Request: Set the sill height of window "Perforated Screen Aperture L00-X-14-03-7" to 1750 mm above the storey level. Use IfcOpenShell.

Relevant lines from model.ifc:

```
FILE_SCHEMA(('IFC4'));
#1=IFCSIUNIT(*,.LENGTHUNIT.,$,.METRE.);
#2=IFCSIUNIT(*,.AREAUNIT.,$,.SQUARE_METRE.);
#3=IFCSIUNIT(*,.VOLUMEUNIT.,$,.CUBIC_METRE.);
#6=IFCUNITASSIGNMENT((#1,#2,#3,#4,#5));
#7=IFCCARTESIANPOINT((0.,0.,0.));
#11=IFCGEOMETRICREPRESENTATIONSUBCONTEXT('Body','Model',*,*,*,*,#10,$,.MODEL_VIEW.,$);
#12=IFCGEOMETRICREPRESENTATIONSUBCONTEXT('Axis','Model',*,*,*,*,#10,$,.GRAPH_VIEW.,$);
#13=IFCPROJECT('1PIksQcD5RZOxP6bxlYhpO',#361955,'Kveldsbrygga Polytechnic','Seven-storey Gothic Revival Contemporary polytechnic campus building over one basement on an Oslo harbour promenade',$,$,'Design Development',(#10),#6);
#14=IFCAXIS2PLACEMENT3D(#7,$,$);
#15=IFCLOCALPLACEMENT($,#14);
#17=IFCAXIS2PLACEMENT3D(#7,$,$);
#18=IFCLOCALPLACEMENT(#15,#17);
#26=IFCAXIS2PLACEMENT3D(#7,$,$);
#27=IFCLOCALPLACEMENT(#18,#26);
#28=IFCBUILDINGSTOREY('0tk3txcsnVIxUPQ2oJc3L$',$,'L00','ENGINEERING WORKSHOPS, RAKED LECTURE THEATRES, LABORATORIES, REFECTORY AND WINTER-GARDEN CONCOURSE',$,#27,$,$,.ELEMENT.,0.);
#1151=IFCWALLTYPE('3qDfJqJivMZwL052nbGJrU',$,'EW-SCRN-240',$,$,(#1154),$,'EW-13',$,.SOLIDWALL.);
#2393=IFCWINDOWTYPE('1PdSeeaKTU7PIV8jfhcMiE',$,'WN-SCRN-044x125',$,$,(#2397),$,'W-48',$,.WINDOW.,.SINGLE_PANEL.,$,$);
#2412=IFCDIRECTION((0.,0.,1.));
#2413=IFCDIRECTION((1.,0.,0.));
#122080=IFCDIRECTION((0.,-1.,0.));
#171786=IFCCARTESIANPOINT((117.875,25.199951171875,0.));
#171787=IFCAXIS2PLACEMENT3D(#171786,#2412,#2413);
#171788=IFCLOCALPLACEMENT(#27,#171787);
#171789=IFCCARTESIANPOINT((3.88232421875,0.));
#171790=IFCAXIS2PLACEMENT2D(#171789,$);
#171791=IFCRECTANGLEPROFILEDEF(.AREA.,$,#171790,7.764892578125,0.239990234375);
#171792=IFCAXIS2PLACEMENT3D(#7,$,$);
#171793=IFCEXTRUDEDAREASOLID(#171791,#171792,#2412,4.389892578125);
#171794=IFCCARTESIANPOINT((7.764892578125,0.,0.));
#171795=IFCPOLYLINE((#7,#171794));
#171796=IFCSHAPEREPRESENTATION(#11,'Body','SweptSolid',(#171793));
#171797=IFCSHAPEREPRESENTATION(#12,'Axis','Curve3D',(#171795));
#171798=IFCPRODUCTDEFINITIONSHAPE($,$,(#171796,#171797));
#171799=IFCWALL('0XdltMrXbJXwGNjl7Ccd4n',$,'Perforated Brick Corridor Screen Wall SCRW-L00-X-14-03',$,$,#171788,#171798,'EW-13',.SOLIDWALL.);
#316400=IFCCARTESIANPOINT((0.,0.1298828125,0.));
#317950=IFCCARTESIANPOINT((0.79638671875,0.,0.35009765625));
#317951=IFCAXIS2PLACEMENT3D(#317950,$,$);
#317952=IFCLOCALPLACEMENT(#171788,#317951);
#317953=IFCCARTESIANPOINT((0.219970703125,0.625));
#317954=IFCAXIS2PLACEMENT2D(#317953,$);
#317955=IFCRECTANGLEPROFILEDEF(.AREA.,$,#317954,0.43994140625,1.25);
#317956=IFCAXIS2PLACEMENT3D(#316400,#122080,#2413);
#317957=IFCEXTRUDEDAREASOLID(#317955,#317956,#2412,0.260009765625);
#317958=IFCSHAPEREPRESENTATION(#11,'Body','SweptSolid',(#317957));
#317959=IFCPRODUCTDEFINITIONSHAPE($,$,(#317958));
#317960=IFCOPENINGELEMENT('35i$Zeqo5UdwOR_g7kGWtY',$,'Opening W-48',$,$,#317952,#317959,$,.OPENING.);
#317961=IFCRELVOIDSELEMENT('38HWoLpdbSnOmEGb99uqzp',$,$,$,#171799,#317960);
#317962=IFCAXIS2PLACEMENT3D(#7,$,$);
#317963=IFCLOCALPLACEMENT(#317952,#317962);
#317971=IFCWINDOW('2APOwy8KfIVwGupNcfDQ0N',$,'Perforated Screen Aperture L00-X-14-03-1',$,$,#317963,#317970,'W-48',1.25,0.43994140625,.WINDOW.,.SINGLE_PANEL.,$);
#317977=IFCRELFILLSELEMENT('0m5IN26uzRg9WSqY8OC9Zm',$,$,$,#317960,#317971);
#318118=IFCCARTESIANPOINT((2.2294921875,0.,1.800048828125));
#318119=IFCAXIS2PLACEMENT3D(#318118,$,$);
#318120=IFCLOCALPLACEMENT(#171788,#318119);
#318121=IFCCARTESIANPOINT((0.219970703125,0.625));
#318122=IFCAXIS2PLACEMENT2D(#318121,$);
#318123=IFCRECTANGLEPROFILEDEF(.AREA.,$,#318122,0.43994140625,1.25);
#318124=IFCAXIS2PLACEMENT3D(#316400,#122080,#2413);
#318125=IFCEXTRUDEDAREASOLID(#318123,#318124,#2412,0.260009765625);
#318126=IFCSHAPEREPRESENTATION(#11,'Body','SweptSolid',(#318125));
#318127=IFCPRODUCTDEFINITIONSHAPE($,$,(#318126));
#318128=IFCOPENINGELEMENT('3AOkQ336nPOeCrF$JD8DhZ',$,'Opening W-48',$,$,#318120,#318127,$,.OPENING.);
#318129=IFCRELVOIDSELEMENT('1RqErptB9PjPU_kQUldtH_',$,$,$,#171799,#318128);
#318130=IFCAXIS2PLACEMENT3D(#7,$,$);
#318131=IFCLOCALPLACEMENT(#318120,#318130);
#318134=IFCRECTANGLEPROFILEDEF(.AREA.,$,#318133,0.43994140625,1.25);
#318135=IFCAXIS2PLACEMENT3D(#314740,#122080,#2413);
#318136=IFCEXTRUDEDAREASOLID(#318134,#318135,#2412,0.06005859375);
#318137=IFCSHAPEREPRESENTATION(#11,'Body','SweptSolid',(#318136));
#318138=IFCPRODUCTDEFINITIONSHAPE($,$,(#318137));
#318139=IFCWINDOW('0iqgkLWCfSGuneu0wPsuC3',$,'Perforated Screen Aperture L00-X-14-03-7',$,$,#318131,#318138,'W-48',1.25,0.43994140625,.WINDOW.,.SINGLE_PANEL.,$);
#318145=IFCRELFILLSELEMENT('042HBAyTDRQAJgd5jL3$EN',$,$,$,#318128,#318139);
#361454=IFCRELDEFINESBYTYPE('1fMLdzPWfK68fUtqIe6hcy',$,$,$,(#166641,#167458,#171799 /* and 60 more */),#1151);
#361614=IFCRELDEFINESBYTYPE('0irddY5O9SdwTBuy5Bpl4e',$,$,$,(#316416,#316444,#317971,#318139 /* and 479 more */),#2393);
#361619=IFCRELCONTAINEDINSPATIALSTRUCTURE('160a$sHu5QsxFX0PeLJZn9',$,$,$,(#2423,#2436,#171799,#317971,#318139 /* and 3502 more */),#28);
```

```python
import numpy as np
import ifcopenshell
import ifcopenshell.api.geometry
import ifcopenshell.geom
import ifcopenshell.util.element
import ifcopenshell.util.placement
import ifcopenshell.util.shape
import ifcopenshell.util.unit

model = ifcopenshell.open("model.ifc")
unit_scale = ifcopenshell.util.unit.calculate_unit_scale(model)

window = model.by_guid("0iqgkLWCfSGuneu0wPsuC3")
opening = window.FillsVoids[0].RelatingOpeningElement
storey = ifcopenshell.util.element.get_container(window, ifc_class="IfcBuildingStorey")
level = ifcopenshell.util.placement.get_local_placement(storey.ObjectPlacement)[2, 3]

# The opening's origin need not be at the sill, so measure its lowest point.
shape = ifcopenshell.geom.create_shape(ifcopenshell.geom.settings(), opening)
bottom = ifcopenshell.util.shape.get_shape_bottom_elevation(shape, shape.geometry) / unit_scale
dz = level + 1.75 / unit_scale - bottom

shift = np.array([0.0, 0.0, dz])
# The window is placed relative to its opening, so it follows when the opening moves.
matrix = ifcopenshell.util.placement.get_local_placement(opening.ObjectPlacement)
matrix[:3, 3] += shift
ifcopenshell.api.geometry.edit_object_placement(
    model, product=opening, matrix=matrix, is_si=False, should_transform_children=True
)

print(f"moved by {dz * unit_scale:+.3f} m")

model.write("model-out.ifc")
```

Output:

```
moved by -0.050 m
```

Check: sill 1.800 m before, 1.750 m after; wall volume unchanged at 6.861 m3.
